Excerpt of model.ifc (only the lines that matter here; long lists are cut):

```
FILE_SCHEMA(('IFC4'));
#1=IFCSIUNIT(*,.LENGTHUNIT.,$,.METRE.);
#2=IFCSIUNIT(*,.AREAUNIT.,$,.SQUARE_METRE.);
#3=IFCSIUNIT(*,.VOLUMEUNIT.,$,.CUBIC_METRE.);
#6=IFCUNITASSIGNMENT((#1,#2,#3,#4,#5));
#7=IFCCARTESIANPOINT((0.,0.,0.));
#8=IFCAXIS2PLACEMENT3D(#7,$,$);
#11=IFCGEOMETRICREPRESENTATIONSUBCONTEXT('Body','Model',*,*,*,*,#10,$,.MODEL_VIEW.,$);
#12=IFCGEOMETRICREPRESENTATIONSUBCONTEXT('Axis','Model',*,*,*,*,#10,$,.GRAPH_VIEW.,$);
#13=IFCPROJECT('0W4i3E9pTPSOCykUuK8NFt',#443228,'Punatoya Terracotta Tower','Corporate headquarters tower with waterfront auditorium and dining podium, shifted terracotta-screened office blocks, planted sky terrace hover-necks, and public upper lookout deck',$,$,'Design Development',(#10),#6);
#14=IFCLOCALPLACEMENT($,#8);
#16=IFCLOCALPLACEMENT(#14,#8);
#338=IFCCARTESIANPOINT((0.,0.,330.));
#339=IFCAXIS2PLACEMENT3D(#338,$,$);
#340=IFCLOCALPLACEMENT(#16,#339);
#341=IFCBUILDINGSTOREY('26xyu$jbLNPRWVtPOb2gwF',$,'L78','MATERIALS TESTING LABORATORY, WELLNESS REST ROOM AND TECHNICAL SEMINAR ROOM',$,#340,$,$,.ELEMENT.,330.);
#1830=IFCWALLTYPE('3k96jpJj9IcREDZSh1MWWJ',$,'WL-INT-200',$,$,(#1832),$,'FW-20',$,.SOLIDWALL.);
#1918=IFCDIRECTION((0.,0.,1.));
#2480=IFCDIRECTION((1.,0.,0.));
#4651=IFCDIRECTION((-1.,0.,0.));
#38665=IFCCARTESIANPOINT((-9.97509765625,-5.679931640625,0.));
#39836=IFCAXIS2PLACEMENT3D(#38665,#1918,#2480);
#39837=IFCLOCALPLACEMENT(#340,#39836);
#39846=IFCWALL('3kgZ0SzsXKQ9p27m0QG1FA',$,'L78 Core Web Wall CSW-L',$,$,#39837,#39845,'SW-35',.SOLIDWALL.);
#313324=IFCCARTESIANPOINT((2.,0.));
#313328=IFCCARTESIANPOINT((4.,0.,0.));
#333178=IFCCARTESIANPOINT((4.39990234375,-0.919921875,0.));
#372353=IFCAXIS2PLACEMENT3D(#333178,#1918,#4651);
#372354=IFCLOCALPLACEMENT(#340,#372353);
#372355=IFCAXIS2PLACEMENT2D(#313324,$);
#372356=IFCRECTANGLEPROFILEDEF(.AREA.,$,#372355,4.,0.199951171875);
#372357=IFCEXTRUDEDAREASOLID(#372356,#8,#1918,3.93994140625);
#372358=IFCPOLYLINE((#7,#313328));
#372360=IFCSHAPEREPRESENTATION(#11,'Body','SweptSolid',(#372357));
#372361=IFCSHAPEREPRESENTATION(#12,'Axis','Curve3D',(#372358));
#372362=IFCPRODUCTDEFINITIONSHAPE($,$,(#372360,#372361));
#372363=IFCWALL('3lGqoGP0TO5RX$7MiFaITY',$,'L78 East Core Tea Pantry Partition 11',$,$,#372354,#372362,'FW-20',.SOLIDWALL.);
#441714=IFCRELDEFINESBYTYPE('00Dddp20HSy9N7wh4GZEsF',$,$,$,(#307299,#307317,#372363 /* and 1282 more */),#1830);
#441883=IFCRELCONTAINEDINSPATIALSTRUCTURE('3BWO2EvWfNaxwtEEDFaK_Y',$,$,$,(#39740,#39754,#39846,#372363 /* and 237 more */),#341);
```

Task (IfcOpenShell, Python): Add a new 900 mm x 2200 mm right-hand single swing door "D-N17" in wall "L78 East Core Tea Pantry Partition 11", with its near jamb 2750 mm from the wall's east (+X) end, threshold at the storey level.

```python
import numpy as np
import ifcopenshell
import ifcopenshell.api.feature
import ifcopenshell.api.geometry
import ifcopenshell.api.root
import ifcopenshell.api.spatial
import ifcopenshell.geom
import ifcopenshell.util.element
import ifcopenshell.util.placement
import ifcopenshell.util.representation
import ifcopenshell.util.shape
import ifcopenshell.util.unit

model = ifcopenshell.open("model.ifc")
unit_scale = ifcopenshell.util.unit.calculate_unit_scale(model)
settings = ifcopenshell.geom.settings()


def volume(element):
    """Net volume in cubic metres, openings subtracted."""
    shape = ifcopenshell.geom.create_shape(settings, element)
    return ifcopenshell.util.shape.get_volume(shape.geometry)


wall = model.by_id(372363)
storey = ifcopenshell.util.element.get_container(wall, ifc_class="IfcBuildingStorey")
context = ifcopenshell.util.representation.get_context(model, "Model", "Body", "MODEL_VIEW")
before = volume(wall)

width, height, from_end, sill = 0.9, 2.2, 2.75, 0.0  # metres

# The wall runs along its own X axis, and the end named is its -X end.
wall_shape = ifcopenshell.geom.create_shape(settings, wall)
x, y, z = ifcopenshell.util.shape.get_vertices(wall_shape.geometry).T
start = x.min() + from_end
face, thickness = float(y.min()), float(y.max() - y.min())
wall_matrix = ifcopenshell.util.placement.get_local_placement(wall.ObjectPlacement)
level = ifcopenshell.util.placement.get_local_placement(storey.ObjectPlacement)[2, 3]


def in_wall(x, y):
    """Placement at x, y metres in the wall's axes, at sill height."""
    matrix = wall_matrix.copy()
    matrix[:, 3] = wall_matrix @ np.array([x / unit_scale, y / unit_scale, 0.0, 1.0])
    matrix[2, 3] = level + sill / unit_scale
    return matrix


# Opening: a box that overshoots both wall faces by 50 mm.
opening = ifcopenshell.api.root.create_entity(model, ifc_class="IfcOpeningElement", predefined_type="OPENING")
box = ifcopenshell.api.geometry.add_wall_representation(
    model, context=context, length=width, height=height, thickness=thickness + 0.1
)
ifcopenshell.api.geometry.assign_representation(model, product=opening, representation=box)
ifcopenshell.api.geometry.edit_object_placement(model, product=opening, matrix=in_wall(start, face - 0.05), is_si=False)
ifcopenshell.api.feature.add_feature(model, feature=opening, element=wall)

door = ifcopenshell.api.root.create_entity(model, ifc_class="IfcDoor", name="D-N17", predefined_type="DOOR")
door.OverallWidth, door.OverallHeight = width / unit_scale, height / unit_scale
door.OperationType = "SINGLE_SWING_RIGHT"
body = ifcopenshell.api.geometry.add_door_representation(
    model,
    context=context,
    overall_width=door.OverallWidth,
    overall_height=door.OverallHeight,
    operation_type="SINGLE_SWING_RIGHT",
    lining_properties={"LiningDepth": thickness / unit_scale, "ThresholdDepth": thickness / unit_scale},
)
ifcopenshell.api.geometry.assign_representation(model, product=door, representation=body)
ifcopenshell.api.spatial.assign_container(model, products=[door], relating_structure=storey)
ifcopenshell.api.feature.add_filling(model, opening=opening, element=door)

# The lining spans the wall, so the door starts at the wall face.
ifcopenshell.api.geometry.edit_object_placement(model, product=door, matrix=in_wall(start, face), is_si=False)

after = volume(wall)

print(f"wall volume {before:.3f} -> {after:.3f} m3")

model.write("model_v2.ifc")
```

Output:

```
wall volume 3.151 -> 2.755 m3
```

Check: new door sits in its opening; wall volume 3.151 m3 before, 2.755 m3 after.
